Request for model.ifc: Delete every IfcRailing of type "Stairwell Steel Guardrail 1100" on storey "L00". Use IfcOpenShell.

First a look at what the model holds.

```python
import ifcopenshell
import ifcopenshell.util.element

model = ifcopenshell.open("model.ifc")
print(model.schema)
storey = next(s for s in model.by_type("IfcBuildingStorey") if s.Name == "L00")
railings = [e for e in ifcopenshell.util.element.get_decomposition(storey) if e.is_a("IfcRailing")]
seen = {}
for e in railings:
    element_type = ifcopenshell.util.element.get_type(e)
    name = element_type.Name if element_type not in (None, e) else None
    seen[name] = seen.get(name, 0) + 1
for name, count in sorted(seen.items(), key=str):
    print(count, "x", name)
```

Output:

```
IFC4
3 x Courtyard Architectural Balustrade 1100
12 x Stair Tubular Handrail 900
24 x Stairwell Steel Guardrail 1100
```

```python
import ifcopenshell
import ifcopenshell.api.root
import ifcopenshell.util.element

model = ifcopenshell.open("model.ifc")

storey = next(s for s in model.by_type("IfcBuildingStorey") if s.Name == "L00")
railings = [e for e in ifcopenshell.util.element.get_decomposition(storey) if e.is_a("IfcRailing")]
targets = [e for e in railings if (t := ifcopenshell.util.element.get_type(e)) not in (None, e) and t.Name == "Stairwell Steel Guardrail 1100"]

for e in targets:
    ifcopenshell.api.root.remove_product(model, product=e)
print(len(targets), "removed")

model.write("model-out.ifc")
```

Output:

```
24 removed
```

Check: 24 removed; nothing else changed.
